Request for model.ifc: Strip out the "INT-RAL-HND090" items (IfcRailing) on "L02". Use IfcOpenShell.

First a look at what the model holds.

```python
import ifcopenshell
import ifcopenshell.util.element

model = ifcopenshell.open("model.ifc")
print(model.schema)
storey = next(s for s in model.by_type("IfcBuildingStorey") if s.Name == "L02")
railings = [e for e in ifcopenshell.util.element.get_decomposition(storey) if e.is_a("IfcRailing")]
seen = {}
for e in railings:
    element_type = ifcopenshell.util.element.get_type(e)
    name = element_type.Name if element_type not in (None, e) else None
    seen[name] = seen.get(name, 0) + 1
for name, count in sorted(seen.items(), key=str):
    print(count, "x", name)
```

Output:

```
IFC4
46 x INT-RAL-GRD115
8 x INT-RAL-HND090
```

```python
import ifcopenshell
import ifcopenshell.api.root
import ifcopenshell.util.element

model = ifcopenshell.open("model.ifc")

storey = next(s for s in model.by_type("IfcBuildingStorey") if s.Name == "L02")
railings = [e for e in ifcopenshell.util.element.get_decomposition(storey) if e.is_a("IfcRailing")]
targets = [e for e in railings if (t := ifcopenshell.util.element.get_type(e)) not in (None, e) and t.Name == "INT-RAL-HND090"]

for e in targets:
    ifcopenshell.api.root.remove_product(model, product=e)
print(len(targets), "removed")

model.write("model_v2.ifc")
```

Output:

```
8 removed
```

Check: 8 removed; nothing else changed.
